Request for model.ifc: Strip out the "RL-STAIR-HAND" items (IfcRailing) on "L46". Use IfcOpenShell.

First a look at what the model holds.

```python
import ifcopenshell
import ifcopenshell.util.element

model = ifcopenshell.open("model.ifc")
print(model.schema)
storey = next(s for s in model.by_type("IfcBuildingStorey") if s.Name == "L46")
railings = [e for e in ifcopenshell.util.element.get_decomposition(storey) if e.is_a("IfcRailing")]
seen = {}
for e in railings:
    element_type = ifcopenshell.util.element.get_type(e)
    name = element_type.Name if element_type not in (None, e) else None
    seen[name] = seen.get(name, 0) + 1
for name, count in sorted(seen.items(), key=str):
    print(count, "x", name)
```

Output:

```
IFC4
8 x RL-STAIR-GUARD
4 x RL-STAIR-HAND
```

```python
import ifcopenshell
import ifcopenshell.api.root
import ifcopenshell.util.element

model = ifcopenshell.open("model.ifc")

storey = next(s for s in model.by_type("IfcBuildingStorey") if s.Name == "L46")
railings = [e for e in ifcopenshell.util.element.get_decomposition(storey) if e.is_a("IfcRailing")]
targets = [e for e in railings if (t := ifcopenshell.util.element.get_type(e)) not in (None, e) and t.Name == "RL-STAIR-HAND"]

for e in targets:
    ifcopenshell.api.root.remove_product(model, product=e)
print(len(targets), "removed")

model.write("model_updated.ifc")
```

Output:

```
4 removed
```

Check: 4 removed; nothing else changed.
